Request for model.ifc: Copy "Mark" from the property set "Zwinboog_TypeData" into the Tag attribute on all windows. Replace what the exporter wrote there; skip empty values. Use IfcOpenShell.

First a look at what the model holds.

```python
import ifcopenshell
import ifcopenshell.util.element

model = ifcopenshell.open("model.ifc")
print(model.schema)
windows = model.by_type("IfcWindow")
print(len(windows), "windows")
for e in windows[:8]:
    source = ifcopenshell.util.element.get_pset(e, "Zwinboog_TypeData", "Mark")
    target = e.Tag
    print(e.id(), repr(source), repr(target), sep=" | ")
```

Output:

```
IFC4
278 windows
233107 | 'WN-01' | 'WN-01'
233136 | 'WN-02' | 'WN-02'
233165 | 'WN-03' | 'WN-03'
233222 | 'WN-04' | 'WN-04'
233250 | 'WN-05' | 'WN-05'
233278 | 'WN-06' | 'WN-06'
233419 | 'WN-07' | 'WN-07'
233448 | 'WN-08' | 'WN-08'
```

```python
import ifcopenshell
import ifcopenshell.util.element

model = ifcopenshell.open("model.ifc")

count = 0
for e in model.by_type("IfcWindow"):
    value = ifcopenshell.util.element.get_pset(e, "Zwinboog_TypeData", "Mark")
    current = e.Tag
    if not value or not value.strip() or current == value:
        continue
    e.Tag = value
    count += 1

print(count, "windows updated")

model.write("model_updated.ifc")
```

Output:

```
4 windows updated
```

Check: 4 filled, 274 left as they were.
